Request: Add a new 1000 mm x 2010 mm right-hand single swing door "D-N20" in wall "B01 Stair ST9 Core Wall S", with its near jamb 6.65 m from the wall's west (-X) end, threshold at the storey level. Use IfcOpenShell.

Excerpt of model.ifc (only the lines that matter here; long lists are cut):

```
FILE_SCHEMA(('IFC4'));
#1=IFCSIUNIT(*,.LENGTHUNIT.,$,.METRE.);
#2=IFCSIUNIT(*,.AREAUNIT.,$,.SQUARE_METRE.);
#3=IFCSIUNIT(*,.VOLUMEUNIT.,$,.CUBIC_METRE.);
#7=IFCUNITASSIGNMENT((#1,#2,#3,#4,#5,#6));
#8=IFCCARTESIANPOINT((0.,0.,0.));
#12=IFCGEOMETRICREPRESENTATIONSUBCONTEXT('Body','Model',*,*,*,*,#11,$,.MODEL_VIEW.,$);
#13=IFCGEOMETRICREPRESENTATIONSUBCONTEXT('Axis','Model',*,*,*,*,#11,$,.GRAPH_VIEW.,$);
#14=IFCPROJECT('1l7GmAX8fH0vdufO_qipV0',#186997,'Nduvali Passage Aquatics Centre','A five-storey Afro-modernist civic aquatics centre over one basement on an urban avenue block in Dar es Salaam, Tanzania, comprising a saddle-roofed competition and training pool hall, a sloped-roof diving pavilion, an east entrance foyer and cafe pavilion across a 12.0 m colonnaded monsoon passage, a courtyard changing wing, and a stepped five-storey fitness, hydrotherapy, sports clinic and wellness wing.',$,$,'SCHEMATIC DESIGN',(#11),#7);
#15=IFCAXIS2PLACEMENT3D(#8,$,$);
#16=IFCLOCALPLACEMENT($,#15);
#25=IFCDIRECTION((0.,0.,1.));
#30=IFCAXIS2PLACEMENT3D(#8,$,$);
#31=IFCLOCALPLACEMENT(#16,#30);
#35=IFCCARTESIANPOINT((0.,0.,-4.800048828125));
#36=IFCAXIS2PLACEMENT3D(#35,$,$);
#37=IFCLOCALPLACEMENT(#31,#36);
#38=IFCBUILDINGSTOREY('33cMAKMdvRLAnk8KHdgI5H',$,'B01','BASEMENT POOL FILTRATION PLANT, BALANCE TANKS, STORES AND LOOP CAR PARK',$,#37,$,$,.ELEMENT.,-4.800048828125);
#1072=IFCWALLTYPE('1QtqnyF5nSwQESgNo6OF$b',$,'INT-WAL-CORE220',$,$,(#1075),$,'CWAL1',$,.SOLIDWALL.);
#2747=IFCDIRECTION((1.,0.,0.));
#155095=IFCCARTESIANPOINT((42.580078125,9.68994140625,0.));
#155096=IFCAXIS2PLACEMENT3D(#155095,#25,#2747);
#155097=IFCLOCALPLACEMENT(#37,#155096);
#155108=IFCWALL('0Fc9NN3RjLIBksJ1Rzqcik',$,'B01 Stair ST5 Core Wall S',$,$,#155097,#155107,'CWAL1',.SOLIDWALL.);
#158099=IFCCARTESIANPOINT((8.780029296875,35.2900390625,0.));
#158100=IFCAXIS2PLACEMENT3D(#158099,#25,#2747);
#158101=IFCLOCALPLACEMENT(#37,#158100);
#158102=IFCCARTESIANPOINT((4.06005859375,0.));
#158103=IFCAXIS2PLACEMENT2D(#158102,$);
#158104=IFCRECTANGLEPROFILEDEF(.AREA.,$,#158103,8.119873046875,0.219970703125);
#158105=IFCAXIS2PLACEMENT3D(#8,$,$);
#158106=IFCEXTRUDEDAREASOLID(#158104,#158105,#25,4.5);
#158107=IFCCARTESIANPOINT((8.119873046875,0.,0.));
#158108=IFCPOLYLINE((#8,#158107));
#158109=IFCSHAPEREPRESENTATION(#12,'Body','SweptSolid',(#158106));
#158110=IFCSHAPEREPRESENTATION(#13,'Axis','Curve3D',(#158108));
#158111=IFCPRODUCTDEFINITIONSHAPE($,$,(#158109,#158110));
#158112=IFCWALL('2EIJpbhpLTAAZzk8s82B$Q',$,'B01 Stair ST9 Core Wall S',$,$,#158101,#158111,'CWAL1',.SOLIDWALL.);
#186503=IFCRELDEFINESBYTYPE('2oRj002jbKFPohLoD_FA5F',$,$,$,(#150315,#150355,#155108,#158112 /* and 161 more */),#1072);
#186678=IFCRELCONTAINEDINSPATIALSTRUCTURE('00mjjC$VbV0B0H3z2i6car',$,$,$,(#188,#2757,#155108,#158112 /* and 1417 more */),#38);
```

```python
import numpy as np
import ifcopenshell
import ifcopenshell.api.feature
import ifcopenshell.api.geometry
import ifcopenshell.api.root
import ifcopenshell.api.spatial
import ifcopenshell.geom
import ifcopenshell.util.element
import ifcopenshell.util.placement
import ifcopenshell.util.representation
import ifcopenshell.util.shape
import ifcopenshell.util.unit

model = ifcopenshell.open("model.ifc")
unit_scale = ifcopenshell.util.unit.calculate_unit_scale(model)
settings = ifcopenshell.geom.settings()


def volume(element):
    """Net volume in cubic metres, openings subtracted."""
    shape = ifcopenshell.geom.create_shape(settings, element)
    return ifcopenshell.util.shape.get_volume(shape.geometry)


wall = model.by_guid("2EIJpbhpLTAAZzk8s82B$Q")
storey = ifcopenshell.util.element.get_container(wall, ifc_class="IfcBuildingStorey")
context = ifcopenshell.util.representation.get_context(model, "Model", "Body", "MODEL_VIEW")
before = volume(wall)

width, height, from_end, sill = 1, 2.01, 6.65, 0.0  # metres

# The wall runs along its own X axis, and the end named is its -X end.
wall_shape = ifcopenshell.geom.create_shape(settings, wall)
x, y, z = ifcopenshell.util.shape.get_vertices(wall_shape.geometry).T
start = x.min() + from_end
face, thickness = float(y.min()), float(y.max() - y.min())
wall_matrix = ifcopenshell.util.placement.get_local_placement(wall.ObjectPlacement)
level = ifcopenshell.util.placement.get_local_placement(storey.ObjectPlacement)[2, 3]


def in_wall(x, y):
    """Placement at x, y metres in the wall's axes, at sill height."""
    matrix = wall_matrix.copy()
    matrix[:, 3] = wall_matrix @ np.array([x / unit_scale, y / unit_scale, 0.0, 1.0])
    matrix[2, 3] = level + sill / unit_scale
    return matrix


# Opening: a box that overshoots both wall faces by 50 mm.
opening = ifcopenshell.api.root.create_entity(model, ifc_class="IfcOpeningElement", predefined_type="OPENING")
box = ifcopenshell.api.geometry.add_wall_representation(
    model, context=context, length=width, height=height, thickness=thickness + 0.1
)
ifcopenshell.api.geometry.assign_representation(model, product=opening, representation=box)
ifcopenshell.api.geometry.edit_object_placement(model, product=opening, matrix=in_wall(start, face - 0.05), is_si=False)
ifcopenshell.api.feature.add_feature(model, feature=opening, element=wall)

door = ifcopenshell.api.root.create_entity(model, ifc_class="IfcDoor", name="D-N20", predefined_type="DOOR")
door.OverallWidth, door.OverallHeight = width / unit_scale, height / unit_scale
door.OperationType = "SINGLE_SWING_RIGHT"
body = ifcopenshell.api.geometry.add_door_representation(
    model,
    context=context,
    overall_width=door.OverallWidth,
    overall_height=door.OverallHeight,
    operation_type="SINGLE_SWING_RIGHT",
    lining_properties={"LiningDepth": thickness / unit_scale, "ThresholdDepth": thickness / unit_scale},
)
ifcopenshell.api.geometry.assign_representation(model, product=door, representation=body)
ifcopenshell.api.spatial.assign_container(model, products=[door], relating_structure=storey)
ifcopenshell.api.feature.add_filling(model, opening=opening, element=door)

# The lining spans the wall, so the door starts at the wall face.
ifcopenshell.api.geometry.edit_object_placement(model, product=door, matrix=in_wall(start, face), is_si=False)

after = volume(wall)

print(f"wall volume {before:.3f} -> {after:.3f} m3")

model.write("model_edited.ifc")
```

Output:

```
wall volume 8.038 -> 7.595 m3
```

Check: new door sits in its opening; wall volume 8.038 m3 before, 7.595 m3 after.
